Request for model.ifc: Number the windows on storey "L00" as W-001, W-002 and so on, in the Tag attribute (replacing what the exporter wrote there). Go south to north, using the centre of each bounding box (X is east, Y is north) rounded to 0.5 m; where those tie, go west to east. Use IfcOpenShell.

First a look at what the model holds.

```python
import ifcopenshell
import ifcopenshell.util.element
import ifcopenshell.util.placement

model = ifcopenshell.open("model.ifc")
print(model.schema)
storey = next(s for s in model.by_type("IfcBuildingStorey") if s.Name == "L00")
windows = [e for e in ifcopenshell.util.element.get_decomposition(storey) if e.is_a("IfcWindow")]
for e in sorted(windows, key=lambda e: e.id()):
    origin = ifcopenshell.util.placement.get_local_placement(e.ObjectPlacement)[:3, 3]
    print(e.id(), e.Tag, e.Name, origin.round(2) + 0.0, sep=" | ")
```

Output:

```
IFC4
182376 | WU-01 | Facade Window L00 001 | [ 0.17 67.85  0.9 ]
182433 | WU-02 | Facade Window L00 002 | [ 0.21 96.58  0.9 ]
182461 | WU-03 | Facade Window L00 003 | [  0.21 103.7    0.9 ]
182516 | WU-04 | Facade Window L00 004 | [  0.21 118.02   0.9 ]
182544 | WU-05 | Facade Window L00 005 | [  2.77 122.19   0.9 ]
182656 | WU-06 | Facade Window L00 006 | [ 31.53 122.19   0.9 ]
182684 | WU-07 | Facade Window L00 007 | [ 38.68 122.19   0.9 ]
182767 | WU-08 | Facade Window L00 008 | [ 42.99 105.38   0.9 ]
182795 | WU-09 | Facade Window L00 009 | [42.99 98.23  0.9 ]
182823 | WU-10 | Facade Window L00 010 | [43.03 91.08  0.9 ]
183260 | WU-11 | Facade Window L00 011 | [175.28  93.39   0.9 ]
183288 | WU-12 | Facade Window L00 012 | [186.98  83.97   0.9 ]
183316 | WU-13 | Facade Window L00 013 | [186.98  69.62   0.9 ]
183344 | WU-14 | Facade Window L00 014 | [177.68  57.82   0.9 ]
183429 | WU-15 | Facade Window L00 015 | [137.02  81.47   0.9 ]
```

```python
import ifcopenshell
import ifcopenshell.geom
import ifcopenshell.util.element
import ifcopenshell.util.shape

model = ifcopenshell.open("model.ifc")
settings = ifcopenshell.geom.settings()
settings.set("use-world-coords", True)


def centre(element):
    shape = ifcopenshell.geom.create_shape(settings, element)
    return ifcopenshell.util.shape.get_bbox_centroid(shape.geometry)


storey = next(s for s in model.by_type("IfcBuildingStorey") if s.Name == "L00")
windows = [e for e in ifcopenshell.util.element.get_decomposition(storey) if e.is_a("IfcWindow")]

# Insertion points can sit at a corner or the storey origin, so sort by the geometry (in metres).
centres = {e: centre(e) for e in windows}
windows.sort(key=lambda e: (round(centres[e][1] / 0.5), centres[e][0]))

for i, e in enumerate(windows, start=1):
    number = f"W-0{i:02d}"
    e.Tag = number
    print(e.id(), number)

model.write("model_v2.ifc")
```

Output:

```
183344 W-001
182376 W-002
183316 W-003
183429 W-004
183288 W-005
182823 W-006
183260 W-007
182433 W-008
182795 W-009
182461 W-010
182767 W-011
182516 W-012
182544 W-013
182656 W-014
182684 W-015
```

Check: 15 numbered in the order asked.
